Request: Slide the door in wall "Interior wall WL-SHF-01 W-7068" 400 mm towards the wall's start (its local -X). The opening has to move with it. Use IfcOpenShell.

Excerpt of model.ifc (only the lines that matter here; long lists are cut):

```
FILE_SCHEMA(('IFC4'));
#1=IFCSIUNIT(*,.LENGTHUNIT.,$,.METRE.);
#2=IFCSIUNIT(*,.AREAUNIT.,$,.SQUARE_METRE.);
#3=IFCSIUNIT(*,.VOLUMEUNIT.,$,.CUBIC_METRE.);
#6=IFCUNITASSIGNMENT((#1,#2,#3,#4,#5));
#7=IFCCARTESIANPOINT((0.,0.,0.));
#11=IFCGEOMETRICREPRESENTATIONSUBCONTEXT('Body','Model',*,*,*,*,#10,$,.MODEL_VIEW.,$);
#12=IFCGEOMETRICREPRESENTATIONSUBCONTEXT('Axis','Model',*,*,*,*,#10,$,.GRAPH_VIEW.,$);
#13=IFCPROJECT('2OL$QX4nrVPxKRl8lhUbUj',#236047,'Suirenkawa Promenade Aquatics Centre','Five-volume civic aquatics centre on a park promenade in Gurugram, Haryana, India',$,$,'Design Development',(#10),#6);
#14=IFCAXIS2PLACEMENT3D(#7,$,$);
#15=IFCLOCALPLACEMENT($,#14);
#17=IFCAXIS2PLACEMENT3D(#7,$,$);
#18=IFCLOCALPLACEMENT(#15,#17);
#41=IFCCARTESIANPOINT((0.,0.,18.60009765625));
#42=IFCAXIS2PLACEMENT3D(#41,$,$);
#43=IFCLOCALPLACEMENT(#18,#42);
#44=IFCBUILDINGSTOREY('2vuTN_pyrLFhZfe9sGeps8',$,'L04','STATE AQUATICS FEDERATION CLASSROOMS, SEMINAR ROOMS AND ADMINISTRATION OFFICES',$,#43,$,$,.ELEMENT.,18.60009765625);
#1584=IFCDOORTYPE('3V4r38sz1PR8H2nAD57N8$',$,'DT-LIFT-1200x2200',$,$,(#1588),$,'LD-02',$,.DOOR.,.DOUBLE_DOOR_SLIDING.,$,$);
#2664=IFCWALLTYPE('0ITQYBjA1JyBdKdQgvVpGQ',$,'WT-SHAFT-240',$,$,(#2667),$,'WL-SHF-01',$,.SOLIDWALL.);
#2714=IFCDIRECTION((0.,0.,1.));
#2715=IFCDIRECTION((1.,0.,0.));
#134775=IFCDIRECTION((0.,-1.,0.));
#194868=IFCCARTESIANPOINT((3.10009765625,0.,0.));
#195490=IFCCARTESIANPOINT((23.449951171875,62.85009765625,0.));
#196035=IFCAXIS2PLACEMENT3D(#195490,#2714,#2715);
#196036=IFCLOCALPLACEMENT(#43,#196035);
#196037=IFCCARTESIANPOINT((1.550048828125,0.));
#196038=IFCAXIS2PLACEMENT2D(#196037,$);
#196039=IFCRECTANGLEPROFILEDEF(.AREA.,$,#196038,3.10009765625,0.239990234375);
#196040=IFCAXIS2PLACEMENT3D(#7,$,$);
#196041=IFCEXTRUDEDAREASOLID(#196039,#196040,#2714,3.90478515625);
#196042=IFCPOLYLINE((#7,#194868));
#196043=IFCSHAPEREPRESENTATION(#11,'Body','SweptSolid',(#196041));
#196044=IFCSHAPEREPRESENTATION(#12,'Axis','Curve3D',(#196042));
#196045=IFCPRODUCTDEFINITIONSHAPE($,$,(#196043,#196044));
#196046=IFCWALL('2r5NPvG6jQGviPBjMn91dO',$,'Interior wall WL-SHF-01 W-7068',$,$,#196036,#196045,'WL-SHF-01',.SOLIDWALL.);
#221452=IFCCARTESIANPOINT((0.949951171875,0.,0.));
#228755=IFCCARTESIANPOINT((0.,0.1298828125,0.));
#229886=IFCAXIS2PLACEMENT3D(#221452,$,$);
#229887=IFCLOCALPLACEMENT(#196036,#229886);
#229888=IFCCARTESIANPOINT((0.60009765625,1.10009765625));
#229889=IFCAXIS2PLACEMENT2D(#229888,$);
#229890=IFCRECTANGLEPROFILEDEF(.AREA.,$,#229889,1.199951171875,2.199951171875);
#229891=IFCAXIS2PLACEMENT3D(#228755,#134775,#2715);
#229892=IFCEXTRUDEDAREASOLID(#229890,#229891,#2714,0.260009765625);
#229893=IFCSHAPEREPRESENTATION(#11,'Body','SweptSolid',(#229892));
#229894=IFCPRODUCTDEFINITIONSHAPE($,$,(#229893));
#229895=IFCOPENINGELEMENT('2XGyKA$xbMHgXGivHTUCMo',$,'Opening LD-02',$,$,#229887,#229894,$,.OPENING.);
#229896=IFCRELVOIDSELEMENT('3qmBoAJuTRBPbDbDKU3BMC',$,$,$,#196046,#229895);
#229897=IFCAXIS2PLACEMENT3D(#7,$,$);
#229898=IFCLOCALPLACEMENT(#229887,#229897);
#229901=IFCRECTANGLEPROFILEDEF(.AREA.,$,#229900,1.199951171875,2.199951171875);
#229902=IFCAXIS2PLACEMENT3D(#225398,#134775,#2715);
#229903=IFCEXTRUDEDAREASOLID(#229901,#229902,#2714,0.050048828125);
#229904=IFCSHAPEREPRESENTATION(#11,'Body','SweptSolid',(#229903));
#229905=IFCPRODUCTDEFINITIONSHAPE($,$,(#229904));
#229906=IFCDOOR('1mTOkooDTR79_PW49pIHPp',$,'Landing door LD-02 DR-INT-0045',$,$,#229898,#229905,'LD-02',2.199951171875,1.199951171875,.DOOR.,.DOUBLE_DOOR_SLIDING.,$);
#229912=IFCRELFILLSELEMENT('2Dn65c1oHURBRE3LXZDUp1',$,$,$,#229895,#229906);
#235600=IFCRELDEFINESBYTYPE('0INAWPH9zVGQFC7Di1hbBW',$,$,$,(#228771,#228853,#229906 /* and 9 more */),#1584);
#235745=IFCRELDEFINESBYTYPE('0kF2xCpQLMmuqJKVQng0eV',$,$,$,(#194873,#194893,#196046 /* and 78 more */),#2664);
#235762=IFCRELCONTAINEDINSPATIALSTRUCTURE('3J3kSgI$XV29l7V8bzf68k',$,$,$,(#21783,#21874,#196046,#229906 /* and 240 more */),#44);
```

```python
import ifcopenshell
import ifcopenshell.api.geometry
import ifcopenshell.util.placement

model = ifcopenshell.open("model.ifc")

door = model.by_id(229906)
opening = door.FillsVoids[0].RelatingOpeningElement
wall = opening.VoidsElements[0].RelatingBuildingElement

wall_matrix = ifcopenshell.util.placement.get_local_placement(wall.ObjectPlacement)
shift = wall_matrix[:3, 0] * -0.4
before = ifcopenshell.util.placement.get_local_placement(door.ObjectPlacement)[:3, 3].copy()

# The door is placed relative to its opening, so it follows when the opening moves.
matrix = ifcopenshell.util.placement.get_local_placement(opening.ObjectPlacement)
matrix[:3, 3] += shift
ifcopenshell.api.geometry.edit_object_placement(
    model, product=opening, matrix=matrix, is_si=False, should_transform_children=True
)

after = ifcopenshell.util.placement.get_local_placement(door.ObjectPlacement)[:3, 3]
print("door moved by", (after - before).round(3) + 0.0)

model.write("model-out.ifc")
```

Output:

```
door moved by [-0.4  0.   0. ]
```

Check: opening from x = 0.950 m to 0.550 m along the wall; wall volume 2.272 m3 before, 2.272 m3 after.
